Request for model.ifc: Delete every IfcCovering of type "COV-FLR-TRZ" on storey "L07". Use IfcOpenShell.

First a look at what the model holds.

```python
import ifcopenshell
import ifcopenshell.util.element

model = ifcopenshell.open("model.ifc")
print(model.schema)
storey = next(s for s in model.by_type("IfcBuildingStorey") if s.Name == "L07")
coverings = [e for e in ifcopenshell.util.element.get_decomposition(storey) if e.is_a("IfcCovering")]
seen = {}
for e in coverings:
    element_type = ifcopenshell.util.element.get_type(e)
    name = element_type.Name if element_type not in (None, e) else None
    seen[name] = seen.get(name, 0) + 1
for name, count in sorted(seen.items(), key=str):
    print(count, "x", name)
```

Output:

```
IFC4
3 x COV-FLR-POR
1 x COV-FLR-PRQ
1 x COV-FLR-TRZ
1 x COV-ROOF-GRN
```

```python
import ifcopenshell
import ifcopenshell.api.root
import ifcopenshell.util.element

model = ifcopenshell.open("model.ifc")

storey = next(s for s in model.by_type("IfcBuildingStorey") if s.Name == "L07")
coverings = [e for e in ifcopenshell.util.element.get_decomposition(storey) if e.is_a("IfcCovering")]
targets = [e for e in coverings if (t := ifcopenshell.util.element.get_type(e)) not in (None, e) and t.Name == "COV-FLR-TRZ"]

for e in targets:
    ifcopenshell.api.root.remove_product(model, product=e)
print(len(targets), "removed")

model.write("model-out.ifc")
```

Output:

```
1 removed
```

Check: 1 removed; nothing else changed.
